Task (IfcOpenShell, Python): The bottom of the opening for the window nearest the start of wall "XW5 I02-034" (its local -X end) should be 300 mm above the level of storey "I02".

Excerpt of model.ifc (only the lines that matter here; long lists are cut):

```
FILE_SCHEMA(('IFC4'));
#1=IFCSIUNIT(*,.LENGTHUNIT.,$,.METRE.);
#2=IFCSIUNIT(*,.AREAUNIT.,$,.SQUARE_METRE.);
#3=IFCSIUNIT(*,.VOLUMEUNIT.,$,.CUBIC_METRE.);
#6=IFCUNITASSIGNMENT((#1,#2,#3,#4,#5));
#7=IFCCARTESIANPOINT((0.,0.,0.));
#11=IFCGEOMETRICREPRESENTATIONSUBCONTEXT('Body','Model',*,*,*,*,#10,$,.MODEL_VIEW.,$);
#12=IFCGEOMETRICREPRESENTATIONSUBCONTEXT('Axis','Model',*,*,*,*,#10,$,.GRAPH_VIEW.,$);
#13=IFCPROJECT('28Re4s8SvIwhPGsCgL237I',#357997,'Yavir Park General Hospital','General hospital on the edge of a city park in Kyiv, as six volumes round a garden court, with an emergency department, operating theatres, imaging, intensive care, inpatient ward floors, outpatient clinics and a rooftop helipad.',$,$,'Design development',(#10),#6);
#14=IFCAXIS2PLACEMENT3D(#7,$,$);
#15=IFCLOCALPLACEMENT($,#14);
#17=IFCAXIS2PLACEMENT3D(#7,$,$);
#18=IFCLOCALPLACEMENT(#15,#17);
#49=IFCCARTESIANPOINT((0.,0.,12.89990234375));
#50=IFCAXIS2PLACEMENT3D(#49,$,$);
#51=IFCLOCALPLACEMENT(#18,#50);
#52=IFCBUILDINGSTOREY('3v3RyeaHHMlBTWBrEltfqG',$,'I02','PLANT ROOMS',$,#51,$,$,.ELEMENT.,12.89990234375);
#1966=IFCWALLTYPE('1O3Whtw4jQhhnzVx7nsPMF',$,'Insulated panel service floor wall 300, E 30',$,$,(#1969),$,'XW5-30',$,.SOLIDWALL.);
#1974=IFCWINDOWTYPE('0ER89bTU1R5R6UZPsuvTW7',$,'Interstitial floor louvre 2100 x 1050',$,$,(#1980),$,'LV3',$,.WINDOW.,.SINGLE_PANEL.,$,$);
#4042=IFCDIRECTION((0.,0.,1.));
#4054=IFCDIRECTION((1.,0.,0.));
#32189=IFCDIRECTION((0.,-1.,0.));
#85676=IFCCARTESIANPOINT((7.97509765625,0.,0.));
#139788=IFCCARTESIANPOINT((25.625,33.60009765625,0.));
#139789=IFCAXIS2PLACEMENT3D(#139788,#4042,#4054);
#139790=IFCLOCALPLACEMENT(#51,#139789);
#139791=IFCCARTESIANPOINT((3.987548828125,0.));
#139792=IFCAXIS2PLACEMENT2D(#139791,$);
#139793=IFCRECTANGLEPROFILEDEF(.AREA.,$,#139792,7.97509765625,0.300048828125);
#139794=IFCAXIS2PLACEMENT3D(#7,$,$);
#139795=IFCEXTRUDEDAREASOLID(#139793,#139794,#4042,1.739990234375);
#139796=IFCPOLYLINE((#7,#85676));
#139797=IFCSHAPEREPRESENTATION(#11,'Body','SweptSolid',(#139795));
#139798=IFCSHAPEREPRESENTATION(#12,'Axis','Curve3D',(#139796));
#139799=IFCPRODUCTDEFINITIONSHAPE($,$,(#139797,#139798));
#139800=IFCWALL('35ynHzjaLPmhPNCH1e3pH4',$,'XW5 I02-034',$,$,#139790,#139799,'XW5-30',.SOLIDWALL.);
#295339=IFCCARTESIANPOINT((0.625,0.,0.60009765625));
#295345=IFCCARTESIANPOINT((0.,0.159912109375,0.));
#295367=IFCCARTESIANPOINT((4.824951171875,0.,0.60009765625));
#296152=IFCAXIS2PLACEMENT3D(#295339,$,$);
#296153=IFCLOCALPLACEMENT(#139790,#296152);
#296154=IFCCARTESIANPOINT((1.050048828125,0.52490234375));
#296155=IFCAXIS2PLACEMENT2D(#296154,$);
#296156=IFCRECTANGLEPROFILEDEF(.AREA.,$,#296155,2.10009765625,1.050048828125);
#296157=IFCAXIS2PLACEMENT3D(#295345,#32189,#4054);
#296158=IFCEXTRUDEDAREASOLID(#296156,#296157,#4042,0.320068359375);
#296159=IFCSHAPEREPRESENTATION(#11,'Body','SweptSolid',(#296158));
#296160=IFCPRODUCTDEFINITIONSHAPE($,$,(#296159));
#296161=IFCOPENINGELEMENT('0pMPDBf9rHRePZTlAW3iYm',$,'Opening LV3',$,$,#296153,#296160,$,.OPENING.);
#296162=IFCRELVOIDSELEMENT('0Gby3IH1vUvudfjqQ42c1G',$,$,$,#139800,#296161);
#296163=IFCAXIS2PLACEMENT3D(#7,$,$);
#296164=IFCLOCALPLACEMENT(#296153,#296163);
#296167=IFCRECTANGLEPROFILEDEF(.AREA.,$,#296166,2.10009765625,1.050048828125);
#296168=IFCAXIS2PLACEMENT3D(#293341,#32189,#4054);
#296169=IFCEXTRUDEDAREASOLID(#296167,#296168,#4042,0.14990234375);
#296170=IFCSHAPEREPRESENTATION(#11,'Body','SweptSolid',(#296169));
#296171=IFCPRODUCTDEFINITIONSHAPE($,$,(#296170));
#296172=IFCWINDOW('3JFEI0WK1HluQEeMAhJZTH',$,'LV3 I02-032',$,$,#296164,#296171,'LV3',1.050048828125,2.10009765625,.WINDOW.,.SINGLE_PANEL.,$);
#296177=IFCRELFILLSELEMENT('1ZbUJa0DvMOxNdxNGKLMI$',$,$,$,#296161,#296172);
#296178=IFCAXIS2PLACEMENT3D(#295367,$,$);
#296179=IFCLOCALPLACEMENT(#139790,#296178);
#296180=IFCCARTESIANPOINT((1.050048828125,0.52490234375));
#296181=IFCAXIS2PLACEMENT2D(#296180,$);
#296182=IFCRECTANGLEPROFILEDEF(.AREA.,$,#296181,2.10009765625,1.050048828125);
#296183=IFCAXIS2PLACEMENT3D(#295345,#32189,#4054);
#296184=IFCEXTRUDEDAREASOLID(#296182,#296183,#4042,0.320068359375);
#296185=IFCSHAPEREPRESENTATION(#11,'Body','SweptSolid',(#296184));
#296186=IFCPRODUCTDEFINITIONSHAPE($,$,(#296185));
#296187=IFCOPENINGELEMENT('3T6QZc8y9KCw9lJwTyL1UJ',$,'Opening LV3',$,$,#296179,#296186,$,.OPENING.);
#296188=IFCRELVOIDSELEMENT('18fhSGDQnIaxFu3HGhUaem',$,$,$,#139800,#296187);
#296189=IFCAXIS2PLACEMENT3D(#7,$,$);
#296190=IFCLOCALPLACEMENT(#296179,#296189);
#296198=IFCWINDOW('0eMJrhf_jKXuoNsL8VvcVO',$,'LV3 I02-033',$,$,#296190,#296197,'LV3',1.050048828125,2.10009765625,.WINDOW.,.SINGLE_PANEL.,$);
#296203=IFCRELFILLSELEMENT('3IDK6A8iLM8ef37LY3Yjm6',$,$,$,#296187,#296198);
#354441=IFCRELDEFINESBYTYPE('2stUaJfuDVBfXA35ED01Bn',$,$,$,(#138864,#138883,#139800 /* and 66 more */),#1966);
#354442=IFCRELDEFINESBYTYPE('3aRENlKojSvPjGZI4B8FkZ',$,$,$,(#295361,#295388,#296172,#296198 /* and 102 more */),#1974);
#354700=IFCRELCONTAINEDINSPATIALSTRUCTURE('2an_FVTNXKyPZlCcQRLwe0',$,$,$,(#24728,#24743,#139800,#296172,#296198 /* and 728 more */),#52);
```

```python
import numpy as np
import ifcopenshell
import ifcopenshell.api.geometry
import ifcopenshell.geom
import ifcopenshell.util.element
import ifcopenshell.util.placement
import ifcopenshell.util.shape
import ifcopenshell.util.unit

model = ifcopenshell.open("model.ifc")
unit_scale = ifcopenshell.util.unit.calculate_unit_scale(model)

window = model.by_guid("3JFEI0WK1HluQEeMAhJZTH")
opening = window.FillsVoids[0].RelatingOpeningElement
storey = ifcopenshell.util.element.get_container(window, ifc_class="IfcBuildingStorey")
level = ifcopenshell.util.placement.get_local_placement(storey.ObjectPlacement)[2, 3]

# The opening's origin need not be at the sill, so measure its lowest point.
shape = ifcopenshell.geom.create_shape(ifcopenshell.geom.settings(), opening)
bottom = ifcopenshell.util.shape.get_shape_bottom_elevation(shape, shape.geometry) / unit_scale
dz = level + 0.3 / unit_scale - bottom

shift = np.array([0.0, 0.0, dz])
# The window is placed relative to its opening, so it follows when the opening moves.
matrix = ifcopenshell.util.placement.get_local_placement(opening.ObjectPlacement)
matrix[:3, 3] += shift
ifcopenshell.api.geometry.edit_object_placement(
    model, product=opening, matrix=matrix, is_si=False, should_transform_children=True
)

print(f"moved by {dz * unit_scale:+.3f} m")

model.write("model_v2.ifc")
```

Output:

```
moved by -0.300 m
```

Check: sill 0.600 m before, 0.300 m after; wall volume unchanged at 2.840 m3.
